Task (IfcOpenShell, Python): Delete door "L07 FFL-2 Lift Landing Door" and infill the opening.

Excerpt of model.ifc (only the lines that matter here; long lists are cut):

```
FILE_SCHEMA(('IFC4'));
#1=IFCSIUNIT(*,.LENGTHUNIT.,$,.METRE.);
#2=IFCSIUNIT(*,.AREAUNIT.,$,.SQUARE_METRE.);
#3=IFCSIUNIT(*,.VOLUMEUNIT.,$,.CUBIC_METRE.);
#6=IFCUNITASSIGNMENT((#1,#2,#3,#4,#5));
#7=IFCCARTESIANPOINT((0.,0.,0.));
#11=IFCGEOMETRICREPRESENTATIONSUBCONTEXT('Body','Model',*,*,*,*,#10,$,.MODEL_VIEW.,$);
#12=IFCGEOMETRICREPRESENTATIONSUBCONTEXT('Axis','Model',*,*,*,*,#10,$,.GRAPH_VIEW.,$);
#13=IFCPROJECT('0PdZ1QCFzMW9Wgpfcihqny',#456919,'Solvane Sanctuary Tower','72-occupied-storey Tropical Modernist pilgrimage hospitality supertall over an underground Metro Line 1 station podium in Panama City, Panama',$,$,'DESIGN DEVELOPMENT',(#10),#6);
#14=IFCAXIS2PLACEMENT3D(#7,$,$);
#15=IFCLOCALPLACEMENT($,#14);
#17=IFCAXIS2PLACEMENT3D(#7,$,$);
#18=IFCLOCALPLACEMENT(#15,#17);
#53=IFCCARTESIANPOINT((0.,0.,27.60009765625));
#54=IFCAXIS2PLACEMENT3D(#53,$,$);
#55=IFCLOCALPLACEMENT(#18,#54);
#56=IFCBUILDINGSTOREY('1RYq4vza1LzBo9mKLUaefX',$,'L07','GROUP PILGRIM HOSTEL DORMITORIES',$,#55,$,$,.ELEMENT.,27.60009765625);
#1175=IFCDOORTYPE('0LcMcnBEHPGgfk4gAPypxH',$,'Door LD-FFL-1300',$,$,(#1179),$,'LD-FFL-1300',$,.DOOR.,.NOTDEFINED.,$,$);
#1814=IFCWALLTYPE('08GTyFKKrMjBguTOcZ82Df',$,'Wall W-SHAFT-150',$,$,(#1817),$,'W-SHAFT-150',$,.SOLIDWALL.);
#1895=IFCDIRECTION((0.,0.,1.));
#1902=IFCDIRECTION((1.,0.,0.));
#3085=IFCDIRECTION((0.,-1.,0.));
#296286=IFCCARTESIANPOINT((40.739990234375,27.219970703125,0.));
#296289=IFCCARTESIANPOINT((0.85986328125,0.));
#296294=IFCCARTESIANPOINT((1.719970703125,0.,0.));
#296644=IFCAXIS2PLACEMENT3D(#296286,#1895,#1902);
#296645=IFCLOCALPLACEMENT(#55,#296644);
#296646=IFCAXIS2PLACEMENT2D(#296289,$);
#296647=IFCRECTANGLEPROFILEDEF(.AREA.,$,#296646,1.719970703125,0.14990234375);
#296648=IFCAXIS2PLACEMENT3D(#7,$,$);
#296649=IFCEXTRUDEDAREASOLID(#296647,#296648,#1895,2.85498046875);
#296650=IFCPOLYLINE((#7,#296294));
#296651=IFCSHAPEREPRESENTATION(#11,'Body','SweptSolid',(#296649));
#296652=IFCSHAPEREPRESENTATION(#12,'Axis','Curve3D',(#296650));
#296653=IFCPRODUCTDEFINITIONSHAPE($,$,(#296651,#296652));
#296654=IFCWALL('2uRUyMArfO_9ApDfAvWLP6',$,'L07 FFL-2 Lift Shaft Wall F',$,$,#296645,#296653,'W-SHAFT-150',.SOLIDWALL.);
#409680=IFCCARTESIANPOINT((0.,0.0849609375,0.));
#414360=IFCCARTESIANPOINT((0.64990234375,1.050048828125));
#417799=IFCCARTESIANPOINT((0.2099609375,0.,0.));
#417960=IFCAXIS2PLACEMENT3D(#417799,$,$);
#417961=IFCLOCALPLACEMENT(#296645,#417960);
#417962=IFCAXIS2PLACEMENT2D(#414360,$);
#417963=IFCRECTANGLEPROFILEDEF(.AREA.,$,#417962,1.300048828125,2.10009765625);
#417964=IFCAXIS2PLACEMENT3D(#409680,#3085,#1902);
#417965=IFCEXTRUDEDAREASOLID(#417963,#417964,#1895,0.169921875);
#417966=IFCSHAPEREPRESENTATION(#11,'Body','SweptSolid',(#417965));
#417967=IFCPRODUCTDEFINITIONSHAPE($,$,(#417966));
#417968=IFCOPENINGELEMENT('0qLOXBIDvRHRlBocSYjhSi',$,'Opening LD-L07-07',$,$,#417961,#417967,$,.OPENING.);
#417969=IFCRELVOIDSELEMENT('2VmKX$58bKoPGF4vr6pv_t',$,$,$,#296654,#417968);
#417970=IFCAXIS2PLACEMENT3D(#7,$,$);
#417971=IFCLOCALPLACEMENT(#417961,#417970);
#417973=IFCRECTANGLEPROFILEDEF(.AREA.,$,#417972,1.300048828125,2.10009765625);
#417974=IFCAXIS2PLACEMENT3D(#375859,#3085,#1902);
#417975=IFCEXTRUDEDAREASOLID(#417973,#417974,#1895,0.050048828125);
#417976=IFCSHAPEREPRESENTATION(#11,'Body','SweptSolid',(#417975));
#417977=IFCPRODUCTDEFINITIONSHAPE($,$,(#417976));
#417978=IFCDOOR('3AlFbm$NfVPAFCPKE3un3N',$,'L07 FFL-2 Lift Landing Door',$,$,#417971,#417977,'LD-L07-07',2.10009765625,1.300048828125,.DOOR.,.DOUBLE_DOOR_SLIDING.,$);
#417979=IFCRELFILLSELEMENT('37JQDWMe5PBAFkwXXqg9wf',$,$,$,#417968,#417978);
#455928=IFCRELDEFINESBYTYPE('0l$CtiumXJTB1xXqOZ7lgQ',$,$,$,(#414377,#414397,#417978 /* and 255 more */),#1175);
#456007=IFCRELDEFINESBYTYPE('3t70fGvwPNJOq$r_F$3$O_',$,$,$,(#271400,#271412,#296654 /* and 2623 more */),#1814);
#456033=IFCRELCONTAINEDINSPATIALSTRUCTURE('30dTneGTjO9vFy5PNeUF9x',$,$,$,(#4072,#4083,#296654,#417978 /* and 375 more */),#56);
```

```python
import ifcopenshell
import ifcopenshell.api.feature
import ifcopenshell.api.root
import ifcopenshell.geom
import ifcopenshell.util.shape

model = ifcopenshell.open("model.ifc")
settings = ifcopenshell.geom.settings()


def volume(element):
    """Net volume in cubic metres, openings subtracted."""
    shape = ifcopenshell.geom.create_shape(settings, element)
    return ifcopenshell.util.shape.get_volume(shape.geometry)


door = model.by_guid("3AlFbm$NfVPAFCPKE3un3N")
opening = door.FillsVoids[0].RelatingOpeningElement
wall = opening.VoidsElements[0].RelatingBuildingElement
before = volume(wall)

ifcopenshell.api.root.remove_product(model, product=door)
ifcopenshell.api.feature.remove_feature(model, feature=opening)

after = volume(wall)

print(f"wall volume {before:.3f} -> {after:.3f} m3")

model.write("model_edited.ifc")
```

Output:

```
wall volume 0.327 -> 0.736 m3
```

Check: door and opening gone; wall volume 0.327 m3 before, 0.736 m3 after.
